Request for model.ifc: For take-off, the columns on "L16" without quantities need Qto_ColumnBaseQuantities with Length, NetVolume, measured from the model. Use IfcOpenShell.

First a look at what the model holds.

```python
import ifcopenshell
import ifcopenshell.util.element
import ifcopenshell.util.unit

model = ifcopenshell.open("model.ifc")
print(model.schema)
for unit_type in ("LENGTHUNIT", "AREAUNIT", "VOLUMEUNIT"):
    print(unit_type, ifcopenshell.util.unit.calculate_unit_scale(model, unit_type))
storey = next(s for s in model.by_type("IfcBuildingStorey") if s.Name == "L16")
columns = [e for e in ifcopenshell.util.element.get_decomposition(storey) if e.is_a("IfcColumn")]
for e in sorted(columns, key=lambda e: e.id()):
    print(e.id(), e.is_a(), e.Name, list(ifcopenshell.util.element.get_psets(e, qtos_only=True)), sep=" | ")
```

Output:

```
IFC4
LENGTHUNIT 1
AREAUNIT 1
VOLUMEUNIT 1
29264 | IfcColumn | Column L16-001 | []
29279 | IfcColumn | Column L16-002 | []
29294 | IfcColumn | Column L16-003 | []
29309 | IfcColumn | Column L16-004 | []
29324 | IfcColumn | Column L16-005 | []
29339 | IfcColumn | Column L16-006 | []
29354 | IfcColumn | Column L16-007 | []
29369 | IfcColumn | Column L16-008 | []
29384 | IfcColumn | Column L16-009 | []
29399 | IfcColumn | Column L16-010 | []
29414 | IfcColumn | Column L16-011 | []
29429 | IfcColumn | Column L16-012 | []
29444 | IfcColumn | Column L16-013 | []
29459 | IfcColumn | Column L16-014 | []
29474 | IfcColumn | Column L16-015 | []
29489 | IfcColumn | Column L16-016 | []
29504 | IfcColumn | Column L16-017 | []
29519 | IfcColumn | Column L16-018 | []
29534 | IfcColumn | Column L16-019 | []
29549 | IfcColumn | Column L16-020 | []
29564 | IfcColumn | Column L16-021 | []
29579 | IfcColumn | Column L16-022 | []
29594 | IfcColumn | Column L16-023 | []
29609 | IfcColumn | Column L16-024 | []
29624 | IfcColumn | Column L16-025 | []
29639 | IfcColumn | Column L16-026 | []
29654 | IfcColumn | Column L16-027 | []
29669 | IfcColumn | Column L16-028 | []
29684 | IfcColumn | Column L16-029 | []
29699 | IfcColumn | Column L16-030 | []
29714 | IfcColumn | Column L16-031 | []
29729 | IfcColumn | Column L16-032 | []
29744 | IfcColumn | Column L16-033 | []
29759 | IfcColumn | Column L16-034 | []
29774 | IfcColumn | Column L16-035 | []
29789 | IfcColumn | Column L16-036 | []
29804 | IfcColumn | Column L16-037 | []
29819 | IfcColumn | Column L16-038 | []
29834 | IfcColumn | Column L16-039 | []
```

```python
import ifcopenshell
import ifcopenshell.api.pset
import ifcopenshell.geom
import ifcopenshell.util.element
import ifcopenshell.util.shape
import ifcopenshell.util.unit

model = ifcopenshell.open("model.ifc")
unit_scale = ifcopenshell.util.unit.calculate_unit_scale(model)
volume_scale = ifcopenshell.util.unit.calculate_unit_scale(model, "VOLUMEUNIT")
settings = ifcopenshell.geom.settings()

storey = next(s for s in model.by_type("IfcBuildingStorey") if s.Name == "L16")
columns = [e for e in ifcopenshell.util.element.get_decomposition(storey) if e.is_a("IfcColumn")]

for e in sorted(columns, key=lambda e: e.id()):
    if ifcopenshell.util.element.get_psets(e, qtos_only=True, should_inherit=False):
        continue
    # Geometry comes back in metres, in the element's own axes.
    shape = ifcopenshell.geom.create_shape(settings, e)
    values = {
        "Length": ifcopenshell.util.shape.get_z(shape.geometry) / unit_scale,
        "NetVolume": ifcopenshell.util.shape.get_volume(shape.geometry) / volume_scale,
    }
    qto = ifcopenshell.api.pset.add_qto(model, product=e, name="Qto_ColumnBaseQuantities")
    ifcopenshell.api.pset.edit_qto(model, qto=qto, properties=values)
    print(e.id(), {k: round(v, 3) for k, v in values.items()})

model.write("model_rev.ifc")
```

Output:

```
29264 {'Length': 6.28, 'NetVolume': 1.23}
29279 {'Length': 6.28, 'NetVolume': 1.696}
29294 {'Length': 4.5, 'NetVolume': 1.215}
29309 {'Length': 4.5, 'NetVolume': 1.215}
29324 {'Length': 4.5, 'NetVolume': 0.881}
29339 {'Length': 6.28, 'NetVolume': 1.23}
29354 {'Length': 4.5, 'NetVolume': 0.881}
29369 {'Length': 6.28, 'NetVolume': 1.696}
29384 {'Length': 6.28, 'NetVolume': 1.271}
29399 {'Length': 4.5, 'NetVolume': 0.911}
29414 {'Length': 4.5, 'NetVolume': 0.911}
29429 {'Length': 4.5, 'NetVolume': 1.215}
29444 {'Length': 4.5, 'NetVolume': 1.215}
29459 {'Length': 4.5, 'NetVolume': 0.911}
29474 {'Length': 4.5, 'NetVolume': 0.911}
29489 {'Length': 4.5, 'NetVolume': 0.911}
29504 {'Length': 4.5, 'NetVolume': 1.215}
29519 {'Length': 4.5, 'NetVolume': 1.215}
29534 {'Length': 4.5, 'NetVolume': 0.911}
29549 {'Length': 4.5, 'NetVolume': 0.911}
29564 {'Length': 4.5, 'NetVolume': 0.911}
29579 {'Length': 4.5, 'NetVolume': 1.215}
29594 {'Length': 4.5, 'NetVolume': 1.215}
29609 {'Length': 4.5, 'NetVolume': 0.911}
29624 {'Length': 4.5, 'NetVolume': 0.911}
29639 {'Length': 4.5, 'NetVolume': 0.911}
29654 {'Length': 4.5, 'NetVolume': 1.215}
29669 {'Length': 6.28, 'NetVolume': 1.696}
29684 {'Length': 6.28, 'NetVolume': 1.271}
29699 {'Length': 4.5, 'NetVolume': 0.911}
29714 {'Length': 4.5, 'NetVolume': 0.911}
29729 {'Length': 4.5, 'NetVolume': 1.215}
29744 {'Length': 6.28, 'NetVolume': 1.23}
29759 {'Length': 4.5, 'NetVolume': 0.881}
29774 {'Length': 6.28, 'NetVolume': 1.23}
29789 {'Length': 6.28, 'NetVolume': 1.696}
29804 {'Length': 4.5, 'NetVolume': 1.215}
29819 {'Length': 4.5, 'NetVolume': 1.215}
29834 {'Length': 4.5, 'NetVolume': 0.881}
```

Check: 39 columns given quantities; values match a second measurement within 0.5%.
